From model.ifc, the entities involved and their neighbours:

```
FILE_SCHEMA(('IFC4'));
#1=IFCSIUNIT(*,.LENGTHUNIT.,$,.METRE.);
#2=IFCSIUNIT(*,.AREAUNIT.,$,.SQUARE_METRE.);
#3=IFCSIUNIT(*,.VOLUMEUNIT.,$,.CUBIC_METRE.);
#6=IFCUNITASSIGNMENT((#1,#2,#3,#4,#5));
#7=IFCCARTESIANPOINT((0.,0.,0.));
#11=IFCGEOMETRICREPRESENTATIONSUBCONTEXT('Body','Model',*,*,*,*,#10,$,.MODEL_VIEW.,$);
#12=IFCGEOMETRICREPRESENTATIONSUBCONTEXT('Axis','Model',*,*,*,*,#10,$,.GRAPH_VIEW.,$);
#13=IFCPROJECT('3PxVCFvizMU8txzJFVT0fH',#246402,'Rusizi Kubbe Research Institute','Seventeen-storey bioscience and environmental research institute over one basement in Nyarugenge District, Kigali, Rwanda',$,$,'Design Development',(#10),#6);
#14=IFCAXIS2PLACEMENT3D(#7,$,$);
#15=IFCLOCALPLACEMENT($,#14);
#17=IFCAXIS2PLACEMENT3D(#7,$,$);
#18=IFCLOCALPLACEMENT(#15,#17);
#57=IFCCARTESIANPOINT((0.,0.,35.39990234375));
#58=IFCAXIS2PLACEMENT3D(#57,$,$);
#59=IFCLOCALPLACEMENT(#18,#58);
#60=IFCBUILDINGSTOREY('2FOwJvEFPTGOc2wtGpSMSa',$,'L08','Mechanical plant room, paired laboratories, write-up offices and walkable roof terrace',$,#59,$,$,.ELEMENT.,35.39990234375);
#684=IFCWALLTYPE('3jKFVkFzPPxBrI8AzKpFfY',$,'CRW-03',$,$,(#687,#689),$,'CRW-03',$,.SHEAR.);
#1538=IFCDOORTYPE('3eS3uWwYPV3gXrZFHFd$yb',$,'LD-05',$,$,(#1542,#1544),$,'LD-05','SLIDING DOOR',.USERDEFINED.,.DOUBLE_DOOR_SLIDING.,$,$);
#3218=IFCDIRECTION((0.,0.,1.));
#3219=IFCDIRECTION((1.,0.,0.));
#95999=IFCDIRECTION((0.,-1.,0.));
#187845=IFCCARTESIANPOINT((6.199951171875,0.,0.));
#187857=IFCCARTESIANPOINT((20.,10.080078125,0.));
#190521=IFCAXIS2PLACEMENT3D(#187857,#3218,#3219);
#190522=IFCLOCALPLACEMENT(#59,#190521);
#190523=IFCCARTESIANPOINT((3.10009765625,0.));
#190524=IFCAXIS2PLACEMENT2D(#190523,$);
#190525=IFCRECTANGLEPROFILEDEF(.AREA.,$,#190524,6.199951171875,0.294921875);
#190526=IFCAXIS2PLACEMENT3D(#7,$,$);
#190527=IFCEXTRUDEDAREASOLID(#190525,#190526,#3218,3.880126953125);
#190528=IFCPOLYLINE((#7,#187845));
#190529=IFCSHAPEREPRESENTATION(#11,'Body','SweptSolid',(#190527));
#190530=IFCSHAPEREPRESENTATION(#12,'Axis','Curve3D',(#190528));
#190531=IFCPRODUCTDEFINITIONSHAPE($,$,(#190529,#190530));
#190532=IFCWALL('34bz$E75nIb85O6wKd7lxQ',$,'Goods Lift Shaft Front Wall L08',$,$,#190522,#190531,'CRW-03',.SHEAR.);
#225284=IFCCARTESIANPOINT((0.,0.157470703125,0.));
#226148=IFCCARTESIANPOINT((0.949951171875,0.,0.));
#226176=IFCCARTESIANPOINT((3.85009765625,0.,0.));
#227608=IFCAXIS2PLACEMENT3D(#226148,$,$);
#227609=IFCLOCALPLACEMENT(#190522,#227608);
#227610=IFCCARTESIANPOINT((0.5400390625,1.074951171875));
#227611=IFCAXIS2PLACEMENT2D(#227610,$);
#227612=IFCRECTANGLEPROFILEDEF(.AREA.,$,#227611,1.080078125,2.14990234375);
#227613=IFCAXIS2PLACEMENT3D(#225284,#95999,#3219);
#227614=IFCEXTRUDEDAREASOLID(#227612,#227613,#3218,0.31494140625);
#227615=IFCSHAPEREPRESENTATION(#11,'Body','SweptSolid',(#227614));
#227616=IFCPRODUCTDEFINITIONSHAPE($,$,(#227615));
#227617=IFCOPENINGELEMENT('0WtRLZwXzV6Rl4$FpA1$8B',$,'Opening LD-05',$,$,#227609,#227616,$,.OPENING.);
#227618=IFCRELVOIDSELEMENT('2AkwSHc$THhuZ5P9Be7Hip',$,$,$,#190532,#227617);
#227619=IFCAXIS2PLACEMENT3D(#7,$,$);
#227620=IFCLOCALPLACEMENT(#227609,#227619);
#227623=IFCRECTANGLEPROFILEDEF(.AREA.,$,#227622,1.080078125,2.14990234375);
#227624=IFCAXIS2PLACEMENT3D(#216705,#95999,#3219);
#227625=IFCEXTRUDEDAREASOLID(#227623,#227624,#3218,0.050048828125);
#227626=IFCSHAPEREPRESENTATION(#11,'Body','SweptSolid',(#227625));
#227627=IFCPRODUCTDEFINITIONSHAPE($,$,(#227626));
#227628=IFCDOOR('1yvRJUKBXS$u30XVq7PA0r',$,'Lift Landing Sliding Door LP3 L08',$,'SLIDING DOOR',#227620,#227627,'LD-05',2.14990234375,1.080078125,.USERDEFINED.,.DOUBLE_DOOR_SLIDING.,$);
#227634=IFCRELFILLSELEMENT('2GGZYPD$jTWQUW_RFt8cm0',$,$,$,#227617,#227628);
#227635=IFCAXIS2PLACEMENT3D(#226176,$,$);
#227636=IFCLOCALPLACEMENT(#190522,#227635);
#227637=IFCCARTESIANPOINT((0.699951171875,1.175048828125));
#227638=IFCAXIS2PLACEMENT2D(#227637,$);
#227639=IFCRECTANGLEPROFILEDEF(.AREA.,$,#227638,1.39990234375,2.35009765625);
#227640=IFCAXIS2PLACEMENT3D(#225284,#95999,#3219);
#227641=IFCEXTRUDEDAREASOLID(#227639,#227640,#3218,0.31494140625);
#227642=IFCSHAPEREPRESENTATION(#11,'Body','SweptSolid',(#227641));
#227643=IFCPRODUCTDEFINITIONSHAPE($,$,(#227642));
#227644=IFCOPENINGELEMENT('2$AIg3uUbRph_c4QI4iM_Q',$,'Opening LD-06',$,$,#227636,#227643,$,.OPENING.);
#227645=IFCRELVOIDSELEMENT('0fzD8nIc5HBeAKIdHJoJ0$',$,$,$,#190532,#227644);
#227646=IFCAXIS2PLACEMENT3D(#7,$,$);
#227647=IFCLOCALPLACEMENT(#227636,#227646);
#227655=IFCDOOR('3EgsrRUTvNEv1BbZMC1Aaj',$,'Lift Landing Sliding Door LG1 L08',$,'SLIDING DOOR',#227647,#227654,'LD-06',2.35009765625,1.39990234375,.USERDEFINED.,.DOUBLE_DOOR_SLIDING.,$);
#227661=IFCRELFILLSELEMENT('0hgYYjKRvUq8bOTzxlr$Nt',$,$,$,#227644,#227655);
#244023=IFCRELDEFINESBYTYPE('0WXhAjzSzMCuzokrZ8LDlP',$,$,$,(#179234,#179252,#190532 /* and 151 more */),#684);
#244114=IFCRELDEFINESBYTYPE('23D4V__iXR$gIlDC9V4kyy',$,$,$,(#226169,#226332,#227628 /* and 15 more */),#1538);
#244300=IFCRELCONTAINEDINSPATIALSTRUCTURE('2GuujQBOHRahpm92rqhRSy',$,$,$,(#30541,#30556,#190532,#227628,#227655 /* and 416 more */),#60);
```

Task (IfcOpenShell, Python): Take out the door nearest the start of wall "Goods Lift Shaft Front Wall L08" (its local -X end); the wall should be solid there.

```python
import ifcopenshell
import ifcopenshell.api.feature
import ifcopenshell.api.root
import ifcopenshell.geom
import ifcopenshell.util.shape

model = ifcopenshell.open("model.ifc")
settings = ifcopenshell.geom.settings()


def volume(element):
    """Net volume in cubic metres, openings subtracted."""
    shape = ifcopenshell.geom.create_shape(settings, element)
    return ifcopenshell.util.shape.get_volume(shape.geometry)


door = model.by_guid("1yvRJUKBXS$u30XVq7PA0r")
opening = door.FillsVoids[0].RelatingOpeningElement
wall = opening.VoidsElements[0].RelatingBuildingElement
before = volume(wall)

ifcopenshell.api.root.remove_product(model, product=door)
ifcopenshell.api.feature.remove_feature(model, feature=opening)

after = volume(wall)

print(f"wall volume {before:.3f} -> {after:.3f} m3")

model.write("model-out.ifc")
```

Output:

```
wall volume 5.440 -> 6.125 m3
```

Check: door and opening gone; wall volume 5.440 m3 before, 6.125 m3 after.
